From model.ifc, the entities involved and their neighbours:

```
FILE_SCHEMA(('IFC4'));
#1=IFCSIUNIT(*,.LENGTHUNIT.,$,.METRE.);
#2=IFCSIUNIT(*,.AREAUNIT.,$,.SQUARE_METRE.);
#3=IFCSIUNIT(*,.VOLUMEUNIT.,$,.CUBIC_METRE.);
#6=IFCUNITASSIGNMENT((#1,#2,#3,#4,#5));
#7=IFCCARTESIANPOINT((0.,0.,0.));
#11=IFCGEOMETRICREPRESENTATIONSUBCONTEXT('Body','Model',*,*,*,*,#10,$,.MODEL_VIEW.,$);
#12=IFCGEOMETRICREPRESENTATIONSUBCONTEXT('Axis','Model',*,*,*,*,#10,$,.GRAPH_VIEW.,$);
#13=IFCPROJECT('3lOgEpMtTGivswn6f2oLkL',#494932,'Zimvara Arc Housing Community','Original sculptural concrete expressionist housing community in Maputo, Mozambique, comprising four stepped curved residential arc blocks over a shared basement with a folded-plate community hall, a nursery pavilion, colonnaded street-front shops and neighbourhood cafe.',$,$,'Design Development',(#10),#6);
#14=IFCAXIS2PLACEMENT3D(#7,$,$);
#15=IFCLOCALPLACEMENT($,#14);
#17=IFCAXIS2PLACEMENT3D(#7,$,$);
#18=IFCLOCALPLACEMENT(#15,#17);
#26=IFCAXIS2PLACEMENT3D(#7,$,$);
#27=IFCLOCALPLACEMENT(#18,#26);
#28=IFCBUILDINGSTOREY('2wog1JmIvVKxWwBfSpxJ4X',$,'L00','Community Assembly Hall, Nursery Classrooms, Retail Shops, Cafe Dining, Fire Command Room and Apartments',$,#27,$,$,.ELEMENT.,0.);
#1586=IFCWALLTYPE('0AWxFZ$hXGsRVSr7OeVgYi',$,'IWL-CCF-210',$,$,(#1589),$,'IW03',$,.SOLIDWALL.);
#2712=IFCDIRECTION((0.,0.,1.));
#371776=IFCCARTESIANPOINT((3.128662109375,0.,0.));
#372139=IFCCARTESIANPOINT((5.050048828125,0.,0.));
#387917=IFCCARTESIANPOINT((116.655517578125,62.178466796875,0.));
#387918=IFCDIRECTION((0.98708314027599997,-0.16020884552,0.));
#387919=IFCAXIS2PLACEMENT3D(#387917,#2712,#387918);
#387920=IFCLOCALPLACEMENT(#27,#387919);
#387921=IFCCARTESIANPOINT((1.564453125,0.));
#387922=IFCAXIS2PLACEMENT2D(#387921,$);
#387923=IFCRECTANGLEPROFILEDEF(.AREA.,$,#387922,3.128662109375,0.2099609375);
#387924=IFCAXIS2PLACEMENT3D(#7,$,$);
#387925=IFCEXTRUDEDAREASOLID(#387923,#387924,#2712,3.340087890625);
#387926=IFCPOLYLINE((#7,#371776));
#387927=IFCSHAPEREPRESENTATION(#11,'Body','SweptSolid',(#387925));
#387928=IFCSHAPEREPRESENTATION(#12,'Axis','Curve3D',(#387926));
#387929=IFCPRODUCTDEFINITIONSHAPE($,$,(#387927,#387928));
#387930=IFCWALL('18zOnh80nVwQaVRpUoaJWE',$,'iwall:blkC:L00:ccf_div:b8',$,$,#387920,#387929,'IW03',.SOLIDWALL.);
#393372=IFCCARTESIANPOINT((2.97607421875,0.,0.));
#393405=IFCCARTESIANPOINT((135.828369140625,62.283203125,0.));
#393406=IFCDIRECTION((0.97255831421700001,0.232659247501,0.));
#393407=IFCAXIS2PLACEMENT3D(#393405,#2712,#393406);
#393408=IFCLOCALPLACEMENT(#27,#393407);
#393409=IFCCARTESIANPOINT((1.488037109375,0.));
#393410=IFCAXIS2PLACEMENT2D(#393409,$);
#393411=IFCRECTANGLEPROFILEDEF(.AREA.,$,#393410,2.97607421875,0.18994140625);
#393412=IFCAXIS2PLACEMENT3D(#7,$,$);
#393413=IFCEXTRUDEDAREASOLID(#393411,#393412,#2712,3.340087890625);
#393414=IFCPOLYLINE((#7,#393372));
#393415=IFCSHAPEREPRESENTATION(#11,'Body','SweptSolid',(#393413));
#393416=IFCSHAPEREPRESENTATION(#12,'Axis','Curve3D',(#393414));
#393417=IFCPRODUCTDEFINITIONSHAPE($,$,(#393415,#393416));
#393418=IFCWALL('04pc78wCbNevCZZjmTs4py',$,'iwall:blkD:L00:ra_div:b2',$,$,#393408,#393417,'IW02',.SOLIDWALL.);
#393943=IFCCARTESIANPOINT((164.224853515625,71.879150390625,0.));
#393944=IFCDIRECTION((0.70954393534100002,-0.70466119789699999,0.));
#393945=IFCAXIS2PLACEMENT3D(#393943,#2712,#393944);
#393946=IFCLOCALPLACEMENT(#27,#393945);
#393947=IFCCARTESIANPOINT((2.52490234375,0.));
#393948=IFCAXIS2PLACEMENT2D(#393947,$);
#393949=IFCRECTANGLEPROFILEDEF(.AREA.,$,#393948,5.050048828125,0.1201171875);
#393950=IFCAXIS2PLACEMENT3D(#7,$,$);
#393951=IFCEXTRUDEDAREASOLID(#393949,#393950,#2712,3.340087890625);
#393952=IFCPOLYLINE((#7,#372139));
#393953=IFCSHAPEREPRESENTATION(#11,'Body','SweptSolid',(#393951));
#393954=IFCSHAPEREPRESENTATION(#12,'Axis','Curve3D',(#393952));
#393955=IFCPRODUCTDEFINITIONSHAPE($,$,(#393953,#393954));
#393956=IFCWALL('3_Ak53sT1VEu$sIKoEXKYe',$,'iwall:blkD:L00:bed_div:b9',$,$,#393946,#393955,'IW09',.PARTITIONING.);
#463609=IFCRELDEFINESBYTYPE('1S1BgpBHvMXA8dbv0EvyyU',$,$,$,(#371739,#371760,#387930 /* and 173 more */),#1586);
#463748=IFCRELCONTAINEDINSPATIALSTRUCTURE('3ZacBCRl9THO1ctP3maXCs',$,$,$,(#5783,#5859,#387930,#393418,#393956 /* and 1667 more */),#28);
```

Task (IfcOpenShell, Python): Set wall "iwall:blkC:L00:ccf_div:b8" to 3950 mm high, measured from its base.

```python
import ifcopenshell
import ifcopenshell.geom
import ifcopenshell.util.representation
import ifcopenshell.util.shape
import ifcopenshell.util.unit

model = ifcopenshell.open("model.ifc")
unit_scale = ifcopenshell.util.unit.calculate_unit_scale(model)
settings = ifcopenshell.geom.settings()


def volume(element):
    """Net volume in cubic metres, openings subtracted."""
    shape = ifcopenshell.geom.create_shape(settings, element)
    return ifcopenshell.util.shape.get_volume(shape.geometry)


wall = model.by_id(387930)
before = volume(wall)

body = ifcopenshell.util.representation.get_representation(wall, "Model", "Body")
solid = body.Items[0]
old_height = solid.Depth
solid.Depth = 3.95 / unit_scale
after = volume(wall)

print(f"height {old_height:g} -> {solid.Depth:g}, volume {before:.3f} -> {after:.3f} m3")

model.write("model_rev.ifc")
```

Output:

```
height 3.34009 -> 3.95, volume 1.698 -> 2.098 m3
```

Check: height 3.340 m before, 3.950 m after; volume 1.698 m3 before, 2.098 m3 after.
